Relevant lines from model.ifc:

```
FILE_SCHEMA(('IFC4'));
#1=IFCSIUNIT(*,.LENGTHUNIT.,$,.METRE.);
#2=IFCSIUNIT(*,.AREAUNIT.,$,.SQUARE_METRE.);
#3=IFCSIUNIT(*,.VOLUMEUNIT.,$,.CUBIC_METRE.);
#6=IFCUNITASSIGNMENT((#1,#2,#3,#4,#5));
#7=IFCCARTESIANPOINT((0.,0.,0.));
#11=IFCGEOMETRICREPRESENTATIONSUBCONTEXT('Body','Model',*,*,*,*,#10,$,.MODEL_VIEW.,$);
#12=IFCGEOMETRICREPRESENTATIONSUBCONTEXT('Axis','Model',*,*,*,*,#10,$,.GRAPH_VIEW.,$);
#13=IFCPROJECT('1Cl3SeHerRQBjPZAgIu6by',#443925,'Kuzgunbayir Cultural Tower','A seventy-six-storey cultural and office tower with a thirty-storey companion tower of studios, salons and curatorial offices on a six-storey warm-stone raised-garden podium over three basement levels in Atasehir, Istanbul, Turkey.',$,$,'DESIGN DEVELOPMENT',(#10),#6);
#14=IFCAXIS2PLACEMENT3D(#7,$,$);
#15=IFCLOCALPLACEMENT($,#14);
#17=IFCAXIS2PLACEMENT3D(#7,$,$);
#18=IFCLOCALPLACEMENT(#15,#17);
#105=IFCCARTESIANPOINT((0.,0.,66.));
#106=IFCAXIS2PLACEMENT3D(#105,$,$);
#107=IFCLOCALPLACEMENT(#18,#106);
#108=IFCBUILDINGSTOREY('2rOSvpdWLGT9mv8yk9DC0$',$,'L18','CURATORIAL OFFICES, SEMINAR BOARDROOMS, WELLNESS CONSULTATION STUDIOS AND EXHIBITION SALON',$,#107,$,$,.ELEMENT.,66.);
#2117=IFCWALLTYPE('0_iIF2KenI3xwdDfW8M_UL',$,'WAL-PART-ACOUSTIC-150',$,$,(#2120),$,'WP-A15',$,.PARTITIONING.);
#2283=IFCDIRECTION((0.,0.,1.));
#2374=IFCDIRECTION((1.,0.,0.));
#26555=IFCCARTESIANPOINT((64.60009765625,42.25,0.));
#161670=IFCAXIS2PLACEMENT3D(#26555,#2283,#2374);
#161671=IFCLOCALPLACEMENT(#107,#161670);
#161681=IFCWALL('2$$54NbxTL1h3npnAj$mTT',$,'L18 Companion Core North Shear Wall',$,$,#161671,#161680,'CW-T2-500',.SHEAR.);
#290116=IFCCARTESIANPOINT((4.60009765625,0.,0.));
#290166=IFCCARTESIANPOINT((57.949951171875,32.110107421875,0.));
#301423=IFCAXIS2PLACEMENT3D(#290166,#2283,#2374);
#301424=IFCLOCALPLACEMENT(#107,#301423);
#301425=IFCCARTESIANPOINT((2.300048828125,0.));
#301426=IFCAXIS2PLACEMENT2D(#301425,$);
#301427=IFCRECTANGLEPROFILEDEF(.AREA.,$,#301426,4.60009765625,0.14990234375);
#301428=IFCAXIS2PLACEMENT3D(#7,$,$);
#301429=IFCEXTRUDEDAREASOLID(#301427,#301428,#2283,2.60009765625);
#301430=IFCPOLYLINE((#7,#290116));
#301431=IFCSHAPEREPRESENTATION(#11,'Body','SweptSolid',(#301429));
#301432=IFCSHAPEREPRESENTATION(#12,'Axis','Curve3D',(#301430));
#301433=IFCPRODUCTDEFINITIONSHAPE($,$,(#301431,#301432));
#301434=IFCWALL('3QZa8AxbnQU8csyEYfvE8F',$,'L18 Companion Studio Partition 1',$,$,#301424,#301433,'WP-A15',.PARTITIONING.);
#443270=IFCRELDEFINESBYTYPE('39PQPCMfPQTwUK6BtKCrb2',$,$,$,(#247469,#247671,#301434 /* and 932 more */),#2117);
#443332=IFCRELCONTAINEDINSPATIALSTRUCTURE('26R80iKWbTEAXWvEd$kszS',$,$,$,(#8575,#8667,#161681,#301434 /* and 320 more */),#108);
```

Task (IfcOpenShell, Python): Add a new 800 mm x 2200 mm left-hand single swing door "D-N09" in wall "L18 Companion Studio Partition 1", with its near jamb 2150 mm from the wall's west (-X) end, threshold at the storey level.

```python
import numpy as np
import ifcopenshell
import ifcopenshell.api.feature
import ifcopenshell.api.geometry
import ifcopenshell.api.root
import ifcopenshell.api.spatial
import ifcopenshell.geom
import ifcopenshell.util.element
import ifcopenshell.util.placement
import ifcopenshell.util.representation
import ifcopenshell.util.shape
import ifcopenshell.util.unit

model = ifcopenshell.open("model.ifc")
unit_scale = ifcopenshell.util.unit.calculate_unit_scale(model)
settings = ifcopenshell.geom.settings()


def volume(element):
    """Net volume in cubic metres, openings subtracted."""
    shape = ifcopenshell.geom.create_shape(settings, element)
    return ifcopenshell.util.shape.get_volume(shape.geometry)


wall = model.by_guid("3QZa8AxbnQU8csyEYfvE8F")
storey = ifcopenshell.util.element.get_container(wall, ifc_class="IfcBuildingStorey")
context = ifcopenshell.util.representation.get_context(model, "Model", "Body", "MODEL_VIEW")
before = volume(wall)

width, height, from_end, sill = 0.8, 2.2, 2.15, 0.0  # metres

# The wall runs along its own X axis, and the end named is its -X end.
wall_shape = ifcopenshell.geom.create_shape(settings, wall)
x, y, z = ifcopenshell.util.shape.get_vertices(wall_shape.geometry).T
start = x.min() + from_end
face, thickness = float(y.min()), float(y.max() - y.min())
wall_matrix = ifcopenshell.util.placement.get_local_placement(wall.ObjectPlacement)
level = ifcopenshell.util.placement.get_local_placement(storey.ObjectPlacement)[2, 3]


def in_wall(x, y):
    """Placement at x, y metres in the wall's axes, at sill height."""
    matrix = wall_matrix.copy()
    matrix[:, 3] = wall_matrix @ np.array([x / unit_scale, y / unit_scale, 0.0, 1.0])
    matrix[2, 3] = level + sill / unit_scale
    return matrix


# Opening: a box that overshoots both wall faces by 50 mm.
opening = ifcopenshell.api.root.create_entity(model, ifc_class="IfcOpeningElement", predefined_type="OPENING")
box = ifcopenshell.api.geometry.add_wall_representation(
    model, context=context, length=width, height=height, thickness=thickness + 0.1
)
ifcopenshell.api.geometry.assign_representation(model, product=opening, representation=box)
ifcopenshell.api.geometry.edit_object_placement(model, product=opening, matrix=in_wall(start, face - 0.05), is_si=False)
ifcopenshell.api.feature.add_feature(model, feature=opening, element=wall)

door = ifcopenshell.api.root.create_entity(model, ifc_class="IfcDoor", name="D-N09", predefined_type="DOOR")
door.OverallWidth, door.OverallHeight = width / unit_scale, height / unit_scale
door.OperationType = "SINGLE_SWING_LEFT"
body = ifcopenshell.api.geometry.add_door_representation(
    model,
    context=context,
    overall_width=door.OverallWidth,
    overall_height=door.OverallHeight,
    operation_type="SINGLE_SWING_LEFT",
    lining_properties={"LiningDepth": thickness / unit_scale, "ThresholdDepth": thickness / unit_scale},
)
ifcopenshell.api.geometry.assign_representation(model, product=door, representation=body)
ifcopenshell.api.spatial.assign_container(model, products=[door], relating_structure=storey)
ifcopenshell.api.feature.add_filling(model, opening=opening, element=door)

# The lining spans the wall, so the door starts at the wall face.
ifcopenshell.api.geometry.edit_object_placement(model, product=door, matrix=in_wall(start, face), is_si=False)

after = volume(wall)

print(f"wall volume {before:.3f} -> {after:.3f} m3")

model.write("model_edited.ifc")
```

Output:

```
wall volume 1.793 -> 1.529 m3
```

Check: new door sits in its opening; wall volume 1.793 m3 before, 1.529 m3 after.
